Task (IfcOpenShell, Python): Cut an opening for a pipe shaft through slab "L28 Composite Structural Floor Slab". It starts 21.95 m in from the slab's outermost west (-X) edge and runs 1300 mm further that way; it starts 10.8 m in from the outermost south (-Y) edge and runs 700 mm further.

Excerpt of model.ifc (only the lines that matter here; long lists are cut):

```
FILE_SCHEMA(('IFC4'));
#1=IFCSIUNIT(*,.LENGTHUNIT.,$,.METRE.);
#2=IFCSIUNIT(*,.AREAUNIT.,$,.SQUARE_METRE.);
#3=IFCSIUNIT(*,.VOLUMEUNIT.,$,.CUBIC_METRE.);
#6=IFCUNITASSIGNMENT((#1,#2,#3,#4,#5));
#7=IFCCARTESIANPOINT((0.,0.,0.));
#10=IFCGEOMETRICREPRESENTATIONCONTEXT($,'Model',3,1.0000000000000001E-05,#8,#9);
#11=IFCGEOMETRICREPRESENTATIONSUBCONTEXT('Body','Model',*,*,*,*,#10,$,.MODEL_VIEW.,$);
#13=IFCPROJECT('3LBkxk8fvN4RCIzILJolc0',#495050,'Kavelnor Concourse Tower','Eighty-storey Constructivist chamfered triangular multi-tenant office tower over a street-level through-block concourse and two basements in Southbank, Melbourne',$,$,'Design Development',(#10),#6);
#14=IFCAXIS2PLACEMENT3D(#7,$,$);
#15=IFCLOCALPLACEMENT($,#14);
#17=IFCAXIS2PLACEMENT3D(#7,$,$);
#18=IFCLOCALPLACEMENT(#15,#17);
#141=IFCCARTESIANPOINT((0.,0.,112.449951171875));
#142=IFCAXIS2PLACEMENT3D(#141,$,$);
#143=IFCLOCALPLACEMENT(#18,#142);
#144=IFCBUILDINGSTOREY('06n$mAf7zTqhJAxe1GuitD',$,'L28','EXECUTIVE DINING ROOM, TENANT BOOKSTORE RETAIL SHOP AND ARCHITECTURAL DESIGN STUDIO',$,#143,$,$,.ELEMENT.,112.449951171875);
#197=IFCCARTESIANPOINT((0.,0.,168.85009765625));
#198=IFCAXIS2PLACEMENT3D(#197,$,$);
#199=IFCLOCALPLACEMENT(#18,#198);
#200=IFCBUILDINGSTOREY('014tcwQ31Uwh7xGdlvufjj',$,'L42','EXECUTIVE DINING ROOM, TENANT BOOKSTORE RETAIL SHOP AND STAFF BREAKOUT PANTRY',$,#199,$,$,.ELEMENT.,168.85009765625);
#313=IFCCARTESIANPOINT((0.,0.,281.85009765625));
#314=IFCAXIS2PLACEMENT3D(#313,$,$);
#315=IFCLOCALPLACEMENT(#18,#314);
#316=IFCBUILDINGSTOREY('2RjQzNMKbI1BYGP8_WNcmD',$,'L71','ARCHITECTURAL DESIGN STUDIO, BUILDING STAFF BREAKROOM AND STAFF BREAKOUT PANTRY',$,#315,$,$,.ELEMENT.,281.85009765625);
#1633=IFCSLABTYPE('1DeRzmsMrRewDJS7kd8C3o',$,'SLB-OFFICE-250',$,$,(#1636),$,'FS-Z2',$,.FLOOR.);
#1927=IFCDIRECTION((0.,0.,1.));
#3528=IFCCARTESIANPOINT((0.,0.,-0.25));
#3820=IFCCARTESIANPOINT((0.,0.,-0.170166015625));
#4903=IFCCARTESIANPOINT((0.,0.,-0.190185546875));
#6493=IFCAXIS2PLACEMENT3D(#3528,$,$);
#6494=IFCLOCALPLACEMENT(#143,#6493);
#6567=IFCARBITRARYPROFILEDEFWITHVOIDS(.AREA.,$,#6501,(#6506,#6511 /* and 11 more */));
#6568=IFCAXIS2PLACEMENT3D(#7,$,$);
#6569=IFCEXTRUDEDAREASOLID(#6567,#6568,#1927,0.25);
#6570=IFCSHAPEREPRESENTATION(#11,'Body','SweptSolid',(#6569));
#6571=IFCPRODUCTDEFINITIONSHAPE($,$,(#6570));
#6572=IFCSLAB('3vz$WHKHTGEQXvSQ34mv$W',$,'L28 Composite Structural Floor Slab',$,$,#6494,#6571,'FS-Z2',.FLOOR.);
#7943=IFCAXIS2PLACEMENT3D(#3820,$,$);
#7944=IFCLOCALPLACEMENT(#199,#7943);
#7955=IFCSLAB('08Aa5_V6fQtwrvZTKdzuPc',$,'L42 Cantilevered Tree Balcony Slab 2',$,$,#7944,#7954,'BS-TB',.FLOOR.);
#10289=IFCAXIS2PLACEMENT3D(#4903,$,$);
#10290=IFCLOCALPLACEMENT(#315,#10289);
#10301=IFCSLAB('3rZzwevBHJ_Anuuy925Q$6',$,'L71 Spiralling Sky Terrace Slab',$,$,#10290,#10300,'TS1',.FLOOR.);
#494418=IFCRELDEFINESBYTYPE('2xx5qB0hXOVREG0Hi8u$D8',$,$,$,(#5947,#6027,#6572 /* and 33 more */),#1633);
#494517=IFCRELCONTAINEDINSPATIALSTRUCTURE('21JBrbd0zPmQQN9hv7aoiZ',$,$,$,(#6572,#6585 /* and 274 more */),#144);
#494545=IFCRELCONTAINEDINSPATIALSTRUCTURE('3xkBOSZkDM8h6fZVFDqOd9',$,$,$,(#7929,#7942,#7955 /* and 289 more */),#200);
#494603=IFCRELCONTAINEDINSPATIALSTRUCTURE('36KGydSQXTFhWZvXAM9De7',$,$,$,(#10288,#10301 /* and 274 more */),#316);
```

```python
import numpy as np
import ifcopenshell
import ifcopenshell.api.feature
import ifcopenshell.api.geometry
import ifcopenshell.api.root
import ifcopenshell.geom
import ifcopenshell.util.placement
import ifcopenshell.util.representation
import ifcopenshell.util.shape
import ifcopenshell.util.unit

model = ifcopenshell.open("model.ifc")
unit_scale = ifcopenshell.util.unit.calculate_unit_scale(model)
settings = ifcopenshell.geom.settings()


def volume(element):
    """Net volume in cubic metres, openings subtracted."""
    shape = ifcopenshell.geom.create_shape(settings, element)
    return ifcopenshell.util.shape.get_volume(shape.geometry)


slab = model.by_guid("3vz$WHKHTGEQXvSQ34mv$W")
before = volume(slab)

# Extent in the slab's own axes, in metres. The edges named are its -X and -Y sides.
slab_shape = ifcopenshell.geom.create_shape(settings, slab)
vertices = ifcopenshell.util.shape.get_vertices(slab_shape.geometry)
x_min, y_min, bottom = vertices.min(axis=0)
top = vertices[:, 2].max()

opening = ifcopenshell.api.root.create_entity(model, ifc_class="IfcOpeningElement", name="Pipe shaft opening", predefined_type="OPENING")
context = ifcopenshell.util.representation.get_context(model, "Model", "Body", "MODEL_VIEW")
width, depth = 1.3, 0.7
outline = [(0.0, 0.0), (width, 0.0), (width, depth), (0.0, depth), (0.0, 0.0)]
# Overshoot both faces by 50 mm so the cut is clean.
shape = ifcopenshell.api.geometry.add_slab_representation(
    model, context=context, depth=top - bottom + 0.1, polyline=outline
)
ifcopenshell.api.geometry.assign_representation(model, product=opening, representation=shape)

matrix = ifcopenshell.util.placement.get_local_placement(slab.ObjectPlacement)
matrix[:, 3] = matrix @ np.append(np.array([x_min + 21.95, y_min + 10.8, bottom - 0.05]) / unit_scale, 1.0)
ifcopenshell.api.geometry.edit_object_placement(model, product=opening, matrix=matrix, is_si=False)
ifcopenshell.api.feature.add_feature(model, feature=opening, element=slab)

after = volume(slab)

print(f"slab volume {before:.3f} -> {after:.3f} m3")

model.write("model_rev.ifc")
```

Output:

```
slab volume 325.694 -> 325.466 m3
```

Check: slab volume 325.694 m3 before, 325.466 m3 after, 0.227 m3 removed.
